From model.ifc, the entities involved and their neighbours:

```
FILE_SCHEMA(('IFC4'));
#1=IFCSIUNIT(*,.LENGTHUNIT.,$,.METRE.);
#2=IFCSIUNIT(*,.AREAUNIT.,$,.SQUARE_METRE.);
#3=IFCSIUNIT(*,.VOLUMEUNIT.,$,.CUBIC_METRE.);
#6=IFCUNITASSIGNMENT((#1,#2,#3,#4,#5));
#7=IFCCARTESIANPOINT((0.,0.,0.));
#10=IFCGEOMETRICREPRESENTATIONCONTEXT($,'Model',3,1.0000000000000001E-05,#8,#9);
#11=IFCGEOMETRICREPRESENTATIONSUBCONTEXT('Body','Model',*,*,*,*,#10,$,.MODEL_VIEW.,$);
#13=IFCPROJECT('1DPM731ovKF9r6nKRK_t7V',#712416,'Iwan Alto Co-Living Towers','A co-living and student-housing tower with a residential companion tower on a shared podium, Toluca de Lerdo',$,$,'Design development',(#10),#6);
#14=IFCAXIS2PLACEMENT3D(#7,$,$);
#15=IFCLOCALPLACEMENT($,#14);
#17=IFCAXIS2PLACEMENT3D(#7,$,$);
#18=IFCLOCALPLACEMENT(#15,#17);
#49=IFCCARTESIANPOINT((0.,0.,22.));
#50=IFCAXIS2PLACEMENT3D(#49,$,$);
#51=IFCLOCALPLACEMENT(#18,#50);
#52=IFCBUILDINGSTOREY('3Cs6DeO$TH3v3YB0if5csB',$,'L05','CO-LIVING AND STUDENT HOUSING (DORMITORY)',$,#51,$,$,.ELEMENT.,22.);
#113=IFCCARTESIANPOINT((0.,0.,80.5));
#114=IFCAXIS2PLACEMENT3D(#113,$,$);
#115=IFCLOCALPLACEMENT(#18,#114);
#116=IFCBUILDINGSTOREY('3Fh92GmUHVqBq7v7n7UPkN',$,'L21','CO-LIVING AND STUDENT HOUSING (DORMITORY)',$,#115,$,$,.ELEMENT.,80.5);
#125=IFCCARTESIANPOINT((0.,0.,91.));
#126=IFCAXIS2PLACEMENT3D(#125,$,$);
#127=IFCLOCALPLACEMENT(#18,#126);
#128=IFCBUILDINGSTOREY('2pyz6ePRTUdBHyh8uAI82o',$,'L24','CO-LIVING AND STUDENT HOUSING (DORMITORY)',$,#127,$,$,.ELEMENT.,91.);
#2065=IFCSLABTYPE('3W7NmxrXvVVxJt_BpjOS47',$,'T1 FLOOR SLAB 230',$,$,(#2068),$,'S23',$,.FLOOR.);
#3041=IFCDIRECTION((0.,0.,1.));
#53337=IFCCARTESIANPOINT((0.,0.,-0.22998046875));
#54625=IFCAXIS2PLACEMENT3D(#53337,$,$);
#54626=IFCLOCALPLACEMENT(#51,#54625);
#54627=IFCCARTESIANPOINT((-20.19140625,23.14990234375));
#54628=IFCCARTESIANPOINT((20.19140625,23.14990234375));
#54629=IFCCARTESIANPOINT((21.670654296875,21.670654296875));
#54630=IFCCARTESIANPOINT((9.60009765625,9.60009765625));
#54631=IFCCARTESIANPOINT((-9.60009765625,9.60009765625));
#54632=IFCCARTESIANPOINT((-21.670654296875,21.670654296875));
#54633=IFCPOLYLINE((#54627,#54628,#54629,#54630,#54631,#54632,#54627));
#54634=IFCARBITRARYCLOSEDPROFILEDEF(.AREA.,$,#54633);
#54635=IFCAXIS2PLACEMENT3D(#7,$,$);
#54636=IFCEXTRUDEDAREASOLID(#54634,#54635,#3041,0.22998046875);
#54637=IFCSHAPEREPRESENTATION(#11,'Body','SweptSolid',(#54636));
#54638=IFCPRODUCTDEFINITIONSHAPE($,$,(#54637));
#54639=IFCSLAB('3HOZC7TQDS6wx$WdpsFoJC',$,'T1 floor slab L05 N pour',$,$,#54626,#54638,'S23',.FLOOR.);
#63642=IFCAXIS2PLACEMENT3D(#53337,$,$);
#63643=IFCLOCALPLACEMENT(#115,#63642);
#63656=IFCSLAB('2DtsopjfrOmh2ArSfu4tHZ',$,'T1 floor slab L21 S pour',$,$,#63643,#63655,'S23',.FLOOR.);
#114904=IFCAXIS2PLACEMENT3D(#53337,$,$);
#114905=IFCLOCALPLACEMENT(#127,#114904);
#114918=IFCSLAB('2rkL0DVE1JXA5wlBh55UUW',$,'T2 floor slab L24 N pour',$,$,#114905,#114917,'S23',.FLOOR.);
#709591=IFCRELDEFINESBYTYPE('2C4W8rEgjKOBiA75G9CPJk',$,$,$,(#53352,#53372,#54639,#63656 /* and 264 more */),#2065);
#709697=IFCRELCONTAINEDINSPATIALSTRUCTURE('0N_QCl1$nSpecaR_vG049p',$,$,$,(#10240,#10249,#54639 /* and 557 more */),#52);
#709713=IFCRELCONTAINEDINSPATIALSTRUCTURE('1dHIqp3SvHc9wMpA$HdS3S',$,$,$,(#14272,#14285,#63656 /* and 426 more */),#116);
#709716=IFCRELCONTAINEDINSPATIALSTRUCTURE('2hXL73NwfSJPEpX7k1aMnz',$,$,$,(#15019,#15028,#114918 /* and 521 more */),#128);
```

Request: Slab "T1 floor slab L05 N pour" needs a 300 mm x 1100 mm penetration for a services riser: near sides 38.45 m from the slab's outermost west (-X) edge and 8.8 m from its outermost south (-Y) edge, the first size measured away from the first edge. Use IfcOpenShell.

```python
import numpy as np
import ifcopenshell
import ifcopenshell.api.feature
import ifcopenshell.api.geometry
import ifcopenshell.api.root
import ifcopenshell.geom
import ifcopenshell.util.placement
import ifcopenshell.util.representation
import ifcopenshell.util.shape
import ifcopenshell.util.unit

model = ifcopenshell.open("model.ifc")
unit_scale = ifcopenshell.util.unit.calculate_unit_scale(model)
settings = ifcopenshell.geom.settings()


def volume(element):
    """Net volume in cubic metres, openings subtracted."""
    shape = ifcopenshell.geom.create_shape(settings, element)
    return ifcopenshell.util.shape.get_volume(shape.geometry)


slab = model.by_id(54639)
before = volume(slab)

# Extent in the slab's own axes, in metres. The edges named are its -X and -Y sides.
slab_shape = ifcopenshell.geom.create_shape(settings, slab)
vertices = ifcopenshell.util.shape.get_vertices(slab_shape.geometry)
x_min, y_min, bottom = vertices.min(axis=0)
top = vertices[:, 2].max()

opening = ifcopenshell.api.root.create_entity(model, ifc_class="IfcOpeningElement", name="Services riser opening", predefined_type="OPENING")
context = ifcopenshell.util.representation.get_context(model, "Model", "Body", "MODEL_VIEW")
width, depth = 0.3, 1.1
outline = [(0.0, 0.0), (width, 0.0), (width, depth), (0.0, depth), (0.0, 0.0)]
# Overshoot both faces by 50 mm so the cut is clean.
shape = ifcopenshell.api.geometry.add_slab_representation(
    model, context=context, depth=top - bottom + 0.1, polyline=outline
)
ifcopenshell.api.geometry.assign_representation(model, product=opening, representation=shape)

matrix = ifcopenshell.util.placement.get_local_placement(slab.ObjectPlacement)
matrix[:, 3] = matrix @ np.append(np.array([x_min + 38.45, y_min + 8.8, bottom - 0.05]) / unit_scale, 1.0)
ifcopenshell.api.geometry.edit_object_placement(model, product=opening, matrix=matrix, is_si=False)
ifcopenshell.api.feature.add_feature(model, feature=opening, element=slab)

after = volume(slab)

print(f"slab volume {before:.3f} -> {after:.3f} m3")

model.write("model_edited.ifc")
```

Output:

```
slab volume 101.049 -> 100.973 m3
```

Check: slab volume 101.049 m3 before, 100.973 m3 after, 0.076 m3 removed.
